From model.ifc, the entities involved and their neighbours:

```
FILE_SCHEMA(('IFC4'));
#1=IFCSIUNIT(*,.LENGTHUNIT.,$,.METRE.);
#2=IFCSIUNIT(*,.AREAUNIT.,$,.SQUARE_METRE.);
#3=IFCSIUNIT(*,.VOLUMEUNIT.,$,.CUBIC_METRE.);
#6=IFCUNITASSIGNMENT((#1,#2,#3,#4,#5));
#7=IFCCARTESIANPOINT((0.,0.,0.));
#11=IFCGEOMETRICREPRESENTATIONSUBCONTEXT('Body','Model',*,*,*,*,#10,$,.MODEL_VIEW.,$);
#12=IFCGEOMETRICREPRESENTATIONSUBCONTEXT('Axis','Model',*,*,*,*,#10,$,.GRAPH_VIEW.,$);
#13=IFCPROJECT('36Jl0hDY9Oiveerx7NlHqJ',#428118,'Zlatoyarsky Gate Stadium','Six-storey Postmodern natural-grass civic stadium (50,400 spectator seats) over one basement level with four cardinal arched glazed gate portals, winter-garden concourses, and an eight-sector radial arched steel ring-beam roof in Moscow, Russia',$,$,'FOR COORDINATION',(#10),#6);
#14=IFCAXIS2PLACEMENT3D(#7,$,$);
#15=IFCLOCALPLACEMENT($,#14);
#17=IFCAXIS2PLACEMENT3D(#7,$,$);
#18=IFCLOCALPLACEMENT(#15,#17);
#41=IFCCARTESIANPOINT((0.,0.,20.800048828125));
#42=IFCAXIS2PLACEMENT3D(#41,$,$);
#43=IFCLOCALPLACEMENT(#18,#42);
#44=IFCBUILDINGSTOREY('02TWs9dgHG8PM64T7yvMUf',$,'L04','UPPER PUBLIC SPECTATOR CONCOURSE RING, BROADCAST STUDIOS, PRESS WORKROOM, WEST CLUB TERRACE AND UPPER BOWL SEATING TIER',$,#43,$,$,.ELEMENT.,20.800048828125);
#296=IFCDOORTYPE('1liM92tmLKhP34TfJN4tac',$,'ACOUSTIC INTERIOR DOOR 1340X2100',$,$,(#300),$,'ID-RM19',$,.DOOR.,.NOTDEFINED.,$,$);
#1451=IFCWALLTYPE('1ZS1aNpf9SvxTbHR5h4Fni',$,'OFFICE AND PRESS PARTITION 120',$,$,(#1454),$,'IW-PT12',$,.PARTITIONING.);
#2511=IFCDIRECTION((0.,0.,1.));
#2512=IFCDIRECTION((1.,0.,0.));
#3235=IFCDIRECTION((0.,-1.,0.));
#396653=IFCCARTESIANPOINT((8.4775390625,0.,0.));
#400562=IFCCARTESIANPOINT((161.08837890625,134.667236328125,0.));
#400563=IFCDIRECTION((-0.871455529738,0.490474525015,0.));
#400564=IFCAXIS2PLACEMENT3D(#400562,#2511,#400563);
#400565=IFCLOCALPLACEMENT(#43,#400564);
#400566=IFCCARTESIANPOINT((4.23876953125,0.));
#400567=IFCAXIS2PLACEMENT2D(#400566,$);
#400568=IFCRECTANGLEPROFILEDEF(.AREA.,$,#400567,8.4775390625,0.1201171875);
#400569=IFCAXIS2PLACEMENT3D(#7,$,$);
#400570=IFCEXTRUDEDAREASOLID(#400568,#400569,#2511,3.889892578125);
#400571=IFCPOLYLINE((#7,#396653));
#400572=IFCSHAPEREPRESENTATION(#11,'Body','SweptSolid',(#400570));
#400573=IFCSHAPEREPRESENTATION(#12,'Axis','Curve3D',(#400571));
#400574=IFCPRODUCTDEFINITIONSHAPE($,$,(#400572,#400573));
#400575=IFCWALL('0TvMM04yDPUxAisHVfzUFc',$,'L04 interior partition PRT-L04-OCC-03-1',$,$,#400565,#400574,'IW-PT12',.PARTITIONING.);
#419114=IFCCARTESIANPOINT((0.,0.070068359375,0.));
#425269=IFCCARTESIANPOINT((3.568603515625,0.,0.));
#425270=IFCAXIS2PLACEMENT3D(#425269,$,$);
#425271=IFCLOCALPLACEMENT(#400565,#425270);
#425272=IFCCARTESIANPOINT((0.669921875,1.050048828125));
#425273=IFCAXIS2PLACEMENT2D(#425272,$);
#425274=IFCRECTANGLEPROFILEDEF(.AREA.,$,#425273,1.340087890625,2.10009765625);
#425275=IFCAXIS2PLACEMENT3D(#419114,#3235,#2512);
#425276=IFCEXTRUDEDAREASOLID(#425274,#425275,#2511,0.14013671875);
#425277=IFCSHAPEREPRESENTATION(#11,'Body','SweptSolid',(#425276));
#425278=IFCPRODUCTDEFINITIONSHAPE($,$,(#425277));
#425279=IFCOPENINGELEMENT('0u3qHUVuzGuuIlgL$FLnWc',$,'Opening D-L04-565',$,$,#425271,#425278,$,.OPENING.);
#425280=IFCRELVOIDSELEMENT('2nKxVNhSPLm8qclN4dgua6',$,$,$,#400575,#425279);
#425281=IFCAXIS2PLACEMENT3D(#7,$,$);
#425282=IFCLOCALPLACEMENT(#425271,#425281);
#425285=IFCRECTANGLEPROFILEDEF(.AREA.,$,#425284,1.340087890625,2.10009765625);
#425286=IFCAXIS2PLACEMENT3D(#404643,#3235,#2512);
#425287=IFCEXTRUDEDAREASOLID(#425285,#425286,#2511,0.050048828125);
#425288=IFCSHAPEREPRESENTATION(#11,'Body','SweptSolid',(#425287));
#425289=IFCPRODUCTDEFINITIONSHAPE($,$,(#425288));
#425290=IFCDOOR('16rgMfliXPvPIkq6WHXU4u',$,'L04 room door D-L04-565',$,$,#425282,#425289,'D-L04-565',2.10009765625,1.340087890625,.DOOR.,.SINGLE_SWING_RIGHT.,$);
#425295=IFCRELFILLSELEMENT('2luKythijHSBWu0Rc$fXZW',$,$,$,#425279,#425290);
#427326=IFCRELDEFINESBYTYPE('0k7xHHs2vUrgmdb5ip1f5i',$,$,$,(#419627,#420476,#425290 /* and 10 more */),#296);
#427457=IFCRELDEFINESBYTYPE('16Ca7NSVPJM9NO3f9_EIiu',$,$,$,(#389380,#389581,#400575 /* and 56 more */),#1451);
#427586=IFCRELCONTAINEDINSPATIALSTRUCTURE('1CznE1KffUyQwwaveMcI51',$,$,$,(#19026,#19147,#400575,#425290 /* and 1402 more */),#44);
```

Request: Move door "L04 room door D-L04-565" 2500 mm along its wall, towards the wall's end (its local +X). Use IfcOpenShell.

```python
import ifcopenshell
import ifcopenshell.api.geometry
import ifcopenshell.util.placement

model = ifcopenshell.open("model.ifc")

door = model.by_guid("16rgMfliXPvPIkq6WHXU4u")
opening = door.FillsVoids[0].RelatingOpeningElement
wall = opening.VoidsElements[0].RelatingBuildingElement

wall_matrix = ifcopenshell.util.placement.get_local_placement(wall.ObjectPlacement)
shift = wall_matrix[:3, 0] * 2.5
before = ifcopenshell.util.placement.get_local_placement(door.ObjectPlacement)[:3, 3].copy()

# The door is placed relative to its opening, so it follows when the opening moves.
matrix = ifcopenshell.util.placement.get_local_placement(opening.ObjectPlacement)
matrix[:3, 3] += shift
ifcopenshell.api.geometry.edit_object_placement(
    model, product=opening, matrix=matrix, is_si=False, should_transform_children=True
)

after = ifcopenshell.util.placement.get_local_placement(door.ObjectPlacement)[:3, 3]
print("door moved by", (after - before).round(3) + 0.0)

model.write("model_v2.ifc")
```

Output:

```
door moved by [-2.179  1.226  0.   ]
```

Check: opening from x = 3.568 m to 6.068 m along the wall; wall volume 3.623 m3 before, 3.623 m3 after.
